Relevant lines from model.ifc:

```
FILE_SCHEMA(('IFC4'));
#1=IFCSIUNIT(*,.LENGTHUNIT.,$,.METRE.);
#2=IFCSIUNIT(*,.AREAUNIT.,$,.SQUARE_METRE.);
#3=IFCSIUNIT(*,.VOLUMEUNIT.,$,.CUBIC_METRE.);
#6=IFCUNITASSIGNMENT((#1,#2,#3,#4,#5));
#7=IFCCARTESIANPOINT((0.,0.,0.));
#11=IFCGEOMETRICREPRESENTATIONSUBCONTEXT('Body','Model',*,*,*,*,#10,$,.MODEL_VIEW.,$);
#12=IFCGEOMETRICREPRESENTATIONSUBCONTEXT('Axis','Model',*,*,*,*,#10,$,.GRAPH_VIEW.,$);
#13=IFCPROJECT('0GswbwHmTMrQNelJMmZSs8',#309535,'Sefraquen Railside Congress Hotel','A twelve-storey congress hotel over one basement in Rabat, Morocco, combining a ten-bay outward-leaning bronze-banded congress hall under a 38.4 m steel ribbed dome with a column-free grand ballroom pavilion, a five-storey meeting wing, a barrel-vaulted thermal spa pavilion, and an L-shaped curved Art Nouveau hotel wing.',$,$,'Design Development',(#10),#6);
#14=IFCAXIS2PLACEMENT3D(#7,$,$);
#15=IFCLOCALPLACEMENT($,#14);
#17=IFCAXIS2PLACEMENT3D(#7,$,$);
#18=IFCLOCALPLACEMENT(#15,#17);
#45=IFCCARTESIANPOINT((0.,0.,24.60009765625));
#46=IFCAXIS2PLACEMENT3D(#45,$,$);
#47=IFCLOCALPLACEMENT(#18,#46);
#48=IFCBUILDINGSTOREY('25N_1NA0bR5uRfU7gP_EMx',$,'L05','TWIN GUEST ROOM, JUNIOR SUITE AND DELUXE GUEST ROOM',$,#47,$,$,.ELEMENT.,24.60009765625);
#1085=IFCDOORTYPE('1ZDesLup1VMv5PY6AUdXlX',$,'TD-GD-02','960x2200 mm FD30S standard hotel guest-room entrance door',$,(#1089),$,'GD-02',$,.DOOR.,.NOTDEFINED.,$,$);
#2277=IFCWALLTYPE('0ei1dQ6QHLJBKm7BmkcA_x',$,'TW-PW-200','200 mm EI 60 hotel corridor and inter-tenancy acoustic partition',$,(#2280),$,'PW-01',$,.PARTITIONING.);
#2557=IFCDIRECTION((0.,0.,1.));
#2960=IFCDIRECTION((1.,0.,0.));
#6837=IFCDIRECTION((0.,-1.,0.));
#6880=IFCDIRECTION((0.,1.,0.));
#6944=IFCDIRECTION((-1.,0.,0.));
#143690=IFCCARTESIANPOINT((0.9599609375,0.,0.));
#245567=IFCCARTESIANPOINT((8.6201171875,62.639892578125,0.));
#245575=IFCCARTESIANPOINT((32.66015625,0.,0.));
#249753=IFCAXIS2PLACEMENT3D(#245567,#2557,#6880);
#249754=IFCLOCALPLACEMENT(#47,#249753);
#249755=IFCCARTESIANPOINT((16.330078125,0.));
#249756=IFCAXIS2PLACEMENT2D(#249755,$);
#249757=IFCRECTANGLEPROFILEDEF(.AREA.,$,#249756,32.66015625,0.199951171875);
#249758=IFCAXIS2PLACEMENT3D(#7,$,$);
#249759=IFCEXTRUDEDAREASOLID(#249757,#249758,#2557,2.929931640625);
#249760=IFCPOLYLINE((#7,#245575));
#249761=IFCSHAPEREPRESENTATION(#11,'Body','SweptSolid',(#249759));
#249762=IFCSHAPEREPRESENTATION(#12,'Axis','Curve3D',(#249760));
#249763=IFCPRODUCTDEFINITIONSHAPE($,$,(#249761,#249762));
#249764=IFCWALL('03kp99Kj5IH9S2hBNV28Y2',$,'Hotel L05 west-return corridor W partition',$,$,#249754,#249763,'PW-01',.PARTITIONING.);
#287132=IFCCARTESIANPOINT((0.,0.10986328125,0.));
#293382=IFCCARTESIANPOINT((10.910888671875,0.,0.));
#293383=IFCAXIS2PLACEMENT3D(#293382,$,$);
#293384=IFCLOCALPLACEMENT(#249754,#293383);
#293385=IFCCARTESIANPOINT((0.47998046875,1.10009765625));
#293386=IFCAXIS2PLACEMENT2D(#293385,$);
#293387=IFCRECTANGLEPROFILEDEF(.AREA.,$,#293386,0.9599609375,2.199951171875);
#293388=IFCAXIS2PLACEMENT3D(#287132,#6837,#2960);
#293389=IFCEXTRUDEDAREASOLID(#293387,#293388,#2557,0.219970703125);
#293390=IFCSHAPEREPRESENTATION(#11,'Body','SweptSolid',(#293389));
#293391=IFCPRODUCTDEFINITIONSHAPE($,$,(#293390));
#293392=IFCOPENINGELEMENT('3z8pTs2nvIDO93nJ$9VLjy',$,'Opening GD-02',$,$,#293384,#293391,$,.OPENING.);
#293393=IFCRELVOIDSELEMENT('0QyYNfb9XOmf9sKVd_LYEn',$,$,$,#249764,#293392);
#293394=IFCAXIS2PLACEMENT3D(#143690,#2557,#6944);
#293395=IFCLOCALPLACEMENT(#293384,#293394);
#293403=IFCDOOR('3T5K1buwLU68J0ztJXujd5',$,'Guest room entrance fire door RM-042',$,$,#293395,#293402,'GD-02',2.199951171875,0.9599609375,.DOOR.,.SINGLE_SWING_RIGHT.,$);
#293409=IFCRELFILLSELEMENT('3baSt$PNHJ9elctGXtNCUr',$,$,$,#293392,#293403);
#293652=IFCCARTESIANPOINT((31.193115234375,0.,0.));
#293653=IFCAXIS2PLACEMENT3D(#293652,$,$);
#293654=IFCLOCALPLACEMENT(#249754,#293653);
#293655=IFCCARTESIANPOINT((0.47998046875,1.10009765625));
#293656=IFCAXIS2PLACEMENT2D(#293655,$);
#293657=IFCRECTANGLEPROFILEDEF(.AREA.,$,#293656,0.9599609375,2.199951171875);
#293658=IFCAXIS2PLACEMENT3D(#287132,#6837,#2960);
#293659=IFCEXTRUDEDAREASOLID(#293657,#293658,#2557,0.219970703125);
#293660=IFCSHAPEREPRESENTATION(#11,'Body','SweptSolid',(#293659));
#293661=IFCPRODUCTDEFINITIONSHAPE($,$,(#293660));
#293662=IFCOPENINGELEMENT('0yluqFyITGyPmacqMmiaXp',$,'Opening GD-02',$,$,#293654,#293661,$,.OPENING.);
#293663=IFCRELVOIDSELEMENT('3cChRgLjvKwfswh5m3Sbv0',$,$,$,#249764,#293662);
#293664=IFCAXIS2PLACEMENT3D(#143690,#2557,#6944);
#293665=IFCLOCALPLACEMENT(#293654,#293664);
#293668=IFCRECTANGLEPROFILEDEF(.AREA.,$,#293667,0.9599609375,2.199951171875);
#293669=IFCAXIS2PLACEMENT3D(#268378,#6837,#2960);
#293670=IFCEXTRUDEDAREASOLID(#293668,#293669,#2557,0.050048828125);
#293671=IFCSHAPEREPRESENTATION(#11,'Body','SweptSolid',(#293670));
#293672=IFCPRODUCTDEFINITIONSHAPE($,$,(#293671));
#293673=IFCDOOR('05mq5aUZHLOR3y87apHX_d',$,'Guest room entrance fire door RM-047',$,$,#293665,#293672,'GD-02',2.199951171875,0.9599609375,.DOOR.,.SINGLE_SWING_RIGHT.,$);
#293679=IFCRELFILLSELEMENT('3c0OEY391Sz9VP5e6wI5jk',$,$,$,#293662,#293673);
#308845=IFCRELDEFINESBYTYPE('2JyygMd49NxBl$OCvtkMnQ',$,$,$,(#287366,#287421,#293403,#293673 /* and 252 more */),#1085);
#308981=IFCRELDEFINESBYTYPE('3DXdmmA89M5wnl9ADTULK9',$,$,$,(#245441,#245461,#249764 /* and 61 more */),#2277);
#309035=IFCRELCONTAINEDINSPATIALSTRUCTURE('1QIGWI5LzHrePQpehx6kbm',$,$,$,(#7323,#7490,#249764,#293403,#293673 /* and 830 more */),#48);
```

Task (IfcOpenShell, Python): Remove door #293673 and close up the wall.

```python
import ifcopenshell
import ifcopenshell.api.feature
import ifcopenshell.api.root
import ifcopenshell.geom
import ifcopenshell.util.shape

model = ifcopenshell.open("model.ifc")
settings = ifcopenshell.geom.settings()


def volume(element):
    """Net volume in cubic metres, openings subtracted."""
    shape = ifcopenshell.geom.create_shape(settings, element)
    return ifcopenshell.util.shape.get_volume(shape.geometry)


door = model.by_id(293673)
opening = door.FillsVoids[0].RelatingOpeningElement
wall = opening.VoidsElements[0].RelatingBuildingElement
before = volume(wall)

ifcopenshell.api.root.remove_product(model, product=door)
ifcopenshell.api.feature.remove_feature(model, feature=opening)

after = volume(wall)

print(f"wall volume {before:.3f} -> {after:.3f} m3")

model.write("model_v2.ifc")
```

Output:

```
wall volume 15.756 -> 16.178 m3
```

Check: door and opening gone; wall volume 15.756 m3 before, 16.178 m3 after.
